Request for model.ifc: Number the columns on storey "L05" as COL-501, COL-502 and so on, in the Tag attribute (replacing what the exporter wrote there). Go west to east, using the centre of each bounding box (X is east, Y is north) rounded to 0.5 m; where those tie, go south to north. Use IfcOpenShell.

First a look at what the model holds.

```python
import ifcopenshell
import ifcopenshell.util.element
import ifcopenshell.util.placement

model = ifcopenshell.open("model.ifc")
print(model.schema)
storey = next(s for s in model.by_type("IfcBuildingStorey") if s.Name == "L05")
columns = [e for e in ifcopenshell.util.element.get_decomposition(storey) if e.is_a("IfcColumn")]
for e in sorted(columns, key=lambda e: e.id()):
    origin = ifcopenshell.util.placement.get_local_placement(e.ObjectPlacement)[:3, 3]
    print(e.id(), e.Tag, e.Name, origin.round(2) + 0.0, sep=" | ")
```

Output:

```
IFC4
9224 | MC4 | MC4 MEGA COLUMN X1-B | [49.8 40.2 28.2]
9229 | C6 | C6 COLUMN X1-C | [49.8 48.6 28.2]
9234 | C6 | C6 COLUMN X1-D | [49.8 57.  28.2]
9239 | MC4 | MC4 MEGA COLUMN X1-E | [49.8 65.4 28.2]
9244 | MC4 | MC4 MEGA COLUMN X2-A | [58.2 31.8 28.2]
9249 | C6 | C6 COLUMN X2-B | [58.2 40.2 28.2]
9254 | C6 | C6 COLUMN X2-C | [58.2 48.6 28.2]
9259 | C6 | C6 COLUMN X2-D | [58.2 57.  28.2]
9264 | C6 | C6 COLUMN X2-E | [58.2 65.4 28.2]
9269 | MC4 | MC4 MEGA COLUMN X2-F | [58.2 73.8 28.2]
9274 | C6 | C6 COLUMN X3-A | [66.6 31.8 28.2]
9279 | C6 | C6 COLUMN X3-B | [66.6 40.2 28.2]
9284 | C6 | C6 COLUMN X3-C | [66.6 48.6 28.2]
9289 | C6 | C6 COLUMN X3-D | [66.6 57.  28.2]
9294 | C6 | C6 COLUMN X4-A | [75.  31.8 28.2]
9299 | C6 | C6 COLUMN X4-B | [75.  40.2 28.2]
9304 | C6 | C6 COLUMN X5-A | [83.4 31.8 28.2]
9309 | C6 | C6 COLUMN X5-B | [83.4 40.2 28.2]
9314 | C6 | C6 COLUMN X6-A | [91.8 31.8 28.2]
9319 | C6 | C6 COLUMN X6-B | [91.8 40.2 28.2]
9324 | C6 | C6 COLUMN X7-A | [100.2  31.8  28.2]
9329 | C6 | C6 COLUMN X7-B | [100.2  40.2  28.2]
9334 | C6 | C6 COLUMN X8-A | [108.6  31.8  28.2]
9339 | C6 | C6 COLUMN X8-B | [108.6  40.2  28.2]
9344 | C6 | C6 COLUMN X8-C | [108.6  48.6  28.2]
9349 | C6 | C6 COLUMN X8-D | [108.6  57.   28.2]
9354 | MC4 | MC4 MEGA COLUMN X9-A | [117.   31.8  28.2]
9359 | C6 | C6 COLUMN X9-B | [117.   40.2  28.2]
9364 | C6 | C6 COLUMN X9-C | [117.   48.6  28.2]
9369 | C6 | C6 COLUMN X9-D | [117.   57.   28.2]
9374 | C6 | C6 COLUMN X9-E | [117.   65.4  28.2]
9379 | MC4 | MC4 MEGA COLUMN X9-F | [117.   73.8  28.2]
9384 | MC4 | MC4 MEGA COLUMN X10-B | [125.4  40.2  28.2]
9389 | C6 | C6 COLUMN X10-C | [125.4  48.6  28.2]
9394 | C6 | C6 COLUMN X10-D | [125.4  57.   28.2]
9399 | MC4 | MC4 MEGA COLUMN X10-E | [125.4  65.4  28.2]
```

```python
import ifcopenshell
import ifcopenshell.geom
import ifcopenshell.util.element
import ifcopenshell.util.shape

model = ifcopenshell.open("model.ifc")
settings = ifcopenshell.geom.settings()
settings.set("use-world-coords", True)


def centre(element):
    shape = ifcopenshell.geom.create_shape(settings, element)
    return ifcopenshell.util.shape.get_bbox_centroid(shape.geometry)


storey = next(s for s in model.by_type("IfcBuildingStorey") if s.Name == "L05")
columns = [e for e in ifcopenshell.util.element.get_decomposition(storey) if e.is_a("IfcColumn")]

# Insertion points can sit at a corner or the storey origin, so sort by the geometry (in metres).
centres = {e: centre(e) for e in columns}
columns.sort(key=lambda e: (round(centres[e][0] / 0.5), centres[e][1]))

for i, e in enumerate(columns, start=1):
    number = f"COL-5{i:02d}"
    e.Tag = number
    print(e.id(), number)

model.write("model_updated.ifc")
```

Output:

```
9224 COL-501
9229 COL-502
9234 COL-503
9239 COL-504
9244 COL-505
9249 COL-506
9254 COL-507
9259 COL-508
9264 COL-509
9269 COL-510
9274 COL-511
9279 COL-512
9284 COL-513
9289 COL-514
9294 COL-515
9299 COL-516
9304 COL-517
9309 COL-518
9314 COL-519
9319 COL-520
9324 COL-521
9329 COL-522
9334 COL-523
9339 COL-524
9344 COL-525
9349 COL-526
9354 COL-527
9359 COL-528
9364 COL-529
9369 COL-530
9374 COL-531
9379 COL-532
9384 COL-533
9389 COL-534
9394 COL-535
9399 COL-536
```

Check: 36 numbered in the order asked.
